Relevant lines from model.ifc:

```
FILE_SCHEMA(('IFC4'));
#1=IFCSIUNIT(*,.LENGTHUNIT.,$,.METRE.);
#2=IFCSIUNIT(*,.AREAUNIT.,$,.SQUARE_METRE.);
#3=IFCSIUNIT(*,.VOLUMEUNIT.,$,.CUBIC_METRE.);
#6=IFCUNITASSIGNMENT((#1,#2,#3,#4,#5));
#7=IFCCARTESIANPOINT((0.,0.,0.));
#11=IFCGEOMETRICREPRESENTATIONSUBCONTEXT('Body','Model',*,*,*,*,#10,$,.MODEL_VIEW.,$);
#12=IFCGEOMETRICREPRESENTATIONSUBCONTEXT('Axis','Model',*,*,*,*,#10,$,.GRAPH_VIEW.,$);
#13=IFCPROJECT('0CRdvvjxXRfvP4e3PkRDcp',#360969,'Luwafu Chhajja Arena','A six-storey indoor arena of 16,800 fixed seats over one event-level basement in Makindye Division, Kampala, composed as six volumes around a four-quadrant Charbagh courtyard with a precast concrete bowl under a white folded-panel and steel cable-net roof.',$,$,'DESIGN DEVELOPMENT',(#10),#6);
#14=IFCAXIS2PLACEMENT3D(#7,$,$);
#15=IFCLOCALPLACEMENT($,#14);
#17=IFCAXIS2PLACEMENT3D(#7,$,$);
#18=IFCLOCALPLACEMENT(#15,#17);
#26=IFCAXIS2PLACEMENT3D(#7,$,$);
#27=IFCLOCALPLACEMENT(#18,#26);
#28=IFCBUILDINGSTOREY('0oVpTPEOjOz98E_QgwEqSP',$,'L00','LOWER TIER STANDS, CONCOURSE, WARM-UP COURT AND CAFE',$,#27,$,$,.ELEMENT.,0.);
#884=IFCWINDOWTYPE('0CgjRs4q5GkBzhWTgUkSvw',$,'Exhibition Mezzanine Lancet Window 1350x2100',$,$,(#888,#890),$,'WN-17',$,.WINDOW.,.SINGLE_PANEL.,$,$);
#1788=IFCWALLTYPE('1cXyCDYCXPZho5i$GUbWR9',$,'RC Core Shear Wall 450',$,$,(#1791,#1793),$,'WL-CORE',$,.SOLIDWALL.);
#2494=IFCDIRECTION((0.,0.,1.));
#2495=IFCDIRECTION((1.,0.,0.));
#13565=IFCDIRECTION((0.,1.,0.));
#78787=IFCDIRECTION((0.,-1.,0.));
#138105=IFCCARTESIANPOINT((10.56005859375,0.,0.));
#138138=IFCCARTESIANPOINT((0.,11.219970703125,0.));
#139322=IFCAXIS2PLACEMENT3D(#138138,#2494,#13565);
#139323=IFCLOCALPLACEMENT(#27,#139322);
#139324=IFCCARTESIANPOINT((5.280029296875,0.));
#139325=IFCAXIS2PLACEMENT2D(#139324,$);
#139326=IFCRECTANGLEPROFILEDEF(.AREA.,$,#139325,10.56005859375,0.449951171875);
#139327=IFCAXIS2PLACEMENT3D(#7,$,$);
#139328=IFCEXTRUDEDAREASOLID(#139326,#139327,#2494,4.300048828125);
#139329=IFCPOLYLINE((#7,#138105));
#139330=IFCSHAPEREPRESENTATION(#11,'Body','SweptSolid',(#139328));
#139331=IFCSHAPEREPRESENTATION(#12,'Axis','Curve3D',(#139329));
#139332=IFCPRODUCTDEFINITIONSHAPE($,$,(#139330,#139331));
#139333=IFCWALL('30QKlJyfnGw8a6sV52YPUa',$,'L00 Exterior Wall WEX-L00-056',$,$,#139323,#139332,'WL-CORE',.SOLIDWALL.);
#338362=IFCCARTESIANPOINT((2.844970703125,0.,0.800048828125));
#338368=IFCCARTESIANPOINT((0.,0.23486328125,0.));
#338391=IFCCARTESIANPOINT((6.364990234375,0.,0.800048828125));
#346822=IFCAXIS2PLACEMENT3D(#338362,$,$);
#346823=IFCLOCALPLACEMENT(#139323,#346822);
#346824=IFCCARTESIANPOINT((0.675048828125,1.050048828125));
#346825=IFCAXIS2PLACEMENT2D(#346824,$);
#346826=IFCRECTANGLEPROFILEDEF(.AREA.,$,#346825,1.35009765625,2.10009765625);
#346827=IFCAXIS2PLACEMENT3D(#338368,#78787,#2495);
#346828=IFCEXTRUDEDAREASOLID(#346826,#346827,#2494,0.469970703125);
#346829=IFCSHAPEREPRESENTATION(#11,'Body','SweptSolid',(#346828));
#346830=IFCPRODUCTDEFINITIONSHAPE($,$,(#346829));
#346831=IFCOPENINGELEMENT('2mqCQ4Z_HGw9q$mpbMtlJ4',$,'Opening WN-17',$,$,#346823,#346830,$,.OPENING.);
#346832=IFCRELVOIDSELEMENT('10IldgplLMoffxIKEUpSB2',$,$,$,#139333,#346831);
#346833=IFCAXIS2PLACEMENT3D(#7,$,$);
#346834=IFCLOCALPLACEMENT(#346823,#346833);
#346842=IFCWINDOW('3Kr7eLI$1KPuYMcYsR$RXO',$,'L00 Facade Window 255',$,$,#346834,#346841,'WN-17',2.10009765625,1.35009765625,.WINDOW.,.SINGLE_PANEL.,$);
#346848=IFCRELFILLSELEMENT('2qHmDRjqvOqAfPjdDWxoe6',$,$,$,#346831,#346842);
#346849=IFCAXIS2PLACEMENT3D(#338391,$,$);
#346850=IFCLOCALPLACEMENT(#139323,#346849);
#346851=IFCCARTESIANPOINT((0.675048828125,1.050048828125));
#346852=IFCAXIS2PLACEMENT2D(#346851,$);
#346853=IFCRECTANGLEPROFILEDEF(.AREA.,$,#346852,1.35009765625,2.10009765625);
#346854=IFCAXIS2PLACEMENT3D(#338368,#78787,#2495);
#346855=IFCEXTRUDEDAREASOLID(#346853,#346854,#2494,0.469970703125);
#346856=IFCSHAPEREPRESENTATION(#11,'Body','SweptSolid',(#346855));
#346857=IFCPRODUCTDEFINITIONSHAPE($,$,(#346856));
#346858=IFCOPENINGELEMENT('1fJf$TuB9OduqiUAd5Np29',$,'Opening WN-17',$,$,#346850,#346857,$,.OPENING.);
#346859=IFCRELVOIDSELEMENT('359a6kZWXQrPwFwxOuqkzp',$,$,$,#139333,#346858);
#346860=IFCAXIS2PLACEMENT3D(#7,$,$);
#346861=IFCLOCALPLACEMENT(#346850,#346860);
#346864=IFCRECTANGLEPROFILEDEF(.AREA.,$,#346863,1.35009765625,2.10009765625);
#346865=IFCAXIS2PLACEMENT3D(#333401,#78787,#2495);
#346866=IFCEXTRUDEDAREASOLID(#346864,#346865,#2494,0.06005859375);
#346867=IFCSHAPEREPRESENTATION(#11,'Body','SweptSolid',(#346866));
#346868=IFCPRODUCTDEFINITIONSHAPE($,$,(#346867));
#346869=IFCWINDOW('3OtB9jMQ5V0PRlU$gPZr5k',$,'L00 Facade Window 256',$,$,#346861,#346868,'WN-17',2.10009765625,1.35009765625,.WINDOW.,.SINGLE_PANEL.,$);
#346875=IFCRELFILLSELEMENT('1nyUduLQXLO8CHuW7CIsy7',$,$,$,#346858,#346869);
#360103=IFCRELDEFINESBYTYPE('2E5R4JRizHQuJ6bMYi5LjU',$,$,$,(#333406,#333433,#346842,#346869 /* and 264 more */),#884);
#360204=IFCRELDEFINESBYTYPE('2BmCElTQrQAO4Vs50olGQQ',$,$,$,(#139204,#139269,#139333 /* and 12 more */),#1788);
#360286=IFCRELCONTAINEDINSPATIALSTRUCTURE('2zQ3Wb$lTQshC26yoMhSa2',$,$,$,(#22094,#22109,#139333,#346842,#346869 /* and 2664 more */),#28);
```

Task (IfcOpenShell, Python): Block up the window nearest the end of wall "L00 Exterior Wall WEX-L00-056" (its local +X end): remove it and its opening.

```python
import ifcopenshell
import ifcopenshell.api.feature
import ifcopenshell.api.root
import ifcopenshell.geom
import ifcopenshell.util.shape

model = ifcopenshell.open("model.ifc")
settings = ifcopenshell.geom.settings()


def volume(element):
    """Net volume in cubic metres, openings subtracted."""
    shape = ifcopenshell.geom.create_shape(settings, element)
    return ifcopenshell.util.shape.get_volume(shape.geometry)


window = model.by_guid("3OtB9jMQ5V0PRlU$gPZr5k")
opening = window.FillsVoids[0].RelatingOpeningElement
wall = opening.VoidsElements[0].RelatingBuildingElement
before = volume(wall)

ifcopenshell.api.root.remove_product(model, product=window)
ifcopenshell.api.feature.remove_feature(model, feature=opening)

after = volume(wall)

print(f"wall volume {before:.3f} -> {after:.3f} m3")

model.write("model_updated.ifc")
```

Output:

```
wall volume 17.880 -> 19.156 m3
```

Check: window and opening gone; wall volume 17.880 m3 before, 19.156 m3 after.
